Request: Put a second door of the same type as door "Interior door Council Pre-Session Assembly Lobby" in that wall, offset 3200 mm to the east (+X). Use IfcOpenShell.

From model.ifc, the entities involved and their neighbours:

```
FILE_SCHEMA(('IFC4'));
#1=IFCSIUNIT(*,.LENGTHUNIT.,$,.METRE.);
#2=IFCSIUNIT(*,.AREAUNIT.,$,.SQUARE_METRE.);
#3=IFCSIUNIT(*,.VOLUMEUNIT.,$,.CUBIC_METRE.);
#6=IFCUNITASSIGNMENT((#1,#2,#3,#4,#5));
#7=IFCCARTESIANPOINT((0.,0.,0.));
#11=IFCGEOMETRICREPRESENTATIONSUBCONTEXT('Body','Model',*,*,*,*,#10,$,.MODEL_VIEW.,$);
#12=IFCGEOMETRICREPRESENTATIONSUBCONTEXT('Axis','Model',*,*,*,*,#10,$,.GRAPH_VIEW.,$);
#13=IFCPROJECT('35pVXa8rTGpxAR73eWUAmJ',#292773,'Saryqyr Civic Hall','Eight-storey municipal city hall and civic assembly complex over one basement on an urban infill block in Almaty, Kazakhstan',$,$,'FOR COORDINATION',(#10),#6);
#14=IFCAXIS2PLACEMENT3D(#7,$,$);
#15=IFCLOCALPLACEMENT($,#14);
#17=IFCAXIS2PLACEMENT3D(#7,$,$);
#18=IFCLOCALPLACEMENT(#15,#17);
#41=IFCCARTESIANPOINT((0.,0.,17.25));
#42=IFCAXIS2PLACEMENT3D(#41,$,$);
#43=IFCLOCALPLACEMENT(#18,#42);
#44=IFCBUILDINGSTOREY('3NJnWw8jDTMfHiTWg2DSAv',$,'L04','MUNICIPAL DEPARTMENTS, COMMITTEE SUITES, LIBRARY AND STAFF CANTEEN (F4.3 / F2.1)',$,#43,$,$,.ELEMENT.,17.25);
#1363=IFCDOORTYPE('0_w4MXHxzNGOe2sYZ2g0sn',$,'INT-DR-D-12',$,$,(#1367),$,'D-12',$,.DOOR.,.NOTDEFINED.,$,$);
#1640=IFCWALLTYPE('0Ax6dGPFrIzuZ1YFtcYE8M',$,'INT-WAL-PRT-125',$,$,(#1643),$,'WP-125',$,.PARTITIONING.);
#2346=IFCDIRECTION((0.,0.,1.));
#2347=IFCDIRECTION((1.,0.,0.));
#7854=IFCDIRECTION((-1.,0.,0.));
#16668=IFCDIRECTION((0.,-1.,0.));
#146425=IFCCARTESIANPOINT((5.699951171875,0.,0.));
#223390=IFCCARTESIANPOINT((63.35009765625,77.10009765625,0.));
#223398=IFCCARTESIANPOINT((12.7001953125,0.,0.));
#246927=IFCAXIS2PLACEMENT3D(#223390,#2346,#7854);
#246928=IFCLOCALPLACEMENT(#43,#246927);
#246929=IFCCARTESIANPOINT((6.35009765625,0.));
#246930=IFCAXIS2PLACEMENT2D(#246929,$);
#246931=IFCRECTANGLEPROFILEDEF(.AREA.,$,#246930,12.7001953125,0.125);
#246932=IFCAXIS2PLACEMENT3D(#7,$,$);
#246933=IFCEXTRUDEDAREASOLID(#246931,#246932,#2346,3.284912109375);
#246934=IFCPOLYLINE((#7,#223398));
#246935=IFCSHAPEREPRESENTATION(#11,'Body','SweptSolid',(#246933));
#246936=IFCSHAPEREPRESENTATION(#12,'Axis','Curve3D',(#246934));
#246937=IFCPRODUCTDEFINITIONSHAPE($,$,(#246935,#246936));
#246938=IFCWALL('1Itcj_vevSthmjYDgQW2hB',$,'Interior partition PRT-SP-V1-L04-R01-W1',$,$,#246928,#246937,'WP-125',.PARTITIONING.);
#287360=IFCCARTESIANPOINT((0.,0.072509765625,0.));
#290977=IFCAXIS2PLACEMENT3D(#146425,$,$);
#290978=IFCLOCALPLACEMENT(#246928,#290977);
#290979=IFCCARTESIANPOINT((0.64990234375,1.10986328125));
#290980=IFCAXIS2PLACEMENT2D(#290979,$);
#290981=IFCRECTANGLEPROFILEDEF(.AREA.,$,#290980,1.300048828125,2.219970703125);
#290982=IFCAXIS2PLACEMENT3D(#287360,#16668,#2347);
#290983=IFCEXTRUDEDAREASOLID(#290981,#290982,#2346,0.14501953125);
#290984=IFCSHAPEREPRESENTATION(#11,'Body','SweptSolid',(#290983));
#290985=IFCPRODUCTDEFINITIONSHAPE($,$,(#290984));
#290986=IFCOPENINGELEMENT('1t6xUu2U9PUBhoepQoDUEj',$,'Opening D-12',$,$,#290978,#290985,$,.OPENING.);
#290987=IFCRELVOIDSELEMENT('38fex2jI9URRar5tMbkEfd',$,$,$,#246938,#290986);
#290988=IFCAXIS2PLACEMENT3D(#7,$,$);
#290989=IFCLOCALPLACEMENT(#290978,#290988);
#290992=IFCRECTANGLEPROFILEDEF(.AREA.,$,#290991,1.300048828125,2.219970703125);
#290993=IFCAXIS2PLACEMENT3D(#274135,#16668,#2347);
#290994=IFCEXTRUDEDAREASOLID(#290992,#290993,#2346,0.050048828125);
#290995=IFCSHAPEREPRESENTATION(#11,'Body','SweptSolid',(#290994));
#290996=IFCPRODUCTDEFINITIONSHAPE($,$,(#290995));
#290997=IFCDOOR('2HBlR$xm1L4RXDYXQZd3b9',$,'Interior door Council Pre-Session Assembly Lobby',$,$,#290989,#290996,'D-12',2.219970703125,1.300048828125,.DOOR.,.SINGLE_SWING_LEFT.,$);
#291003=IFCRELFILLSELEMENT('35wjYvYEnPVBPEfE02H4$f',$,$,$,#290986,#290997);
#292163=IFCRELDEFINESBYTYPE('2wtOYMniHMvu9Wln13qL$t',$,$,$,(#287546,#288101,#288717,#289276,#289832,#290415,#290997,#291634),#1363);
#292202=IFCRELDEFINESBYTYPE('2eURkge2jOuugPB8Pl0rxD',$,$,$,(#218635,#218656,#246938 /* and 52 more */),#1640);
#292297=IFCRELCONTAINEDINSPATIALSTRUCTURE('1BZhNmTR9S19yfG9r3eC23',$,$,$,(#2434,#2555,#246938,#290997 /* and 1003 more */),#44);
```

```python
import ifcopenshell
import ifcopenshell.api.feature
import ifcopenshell.api.geometry
import ifcopenshell.api.root
import ifcopenshell.geom
import ifcopenshell.util.element
import ifcopenshell.util.placement
import ifcopenshell.util.shape
import ifcopenshell.util.unit

model = ifcopenshell.open("model.ifc")
unit_scale = ifcopenshell.util.unit.calculate_unit_scale(model)
settings = ifcopenshell.geom.settings()


def volume(element):
    """Net volume in cubic metres, openings subtracted."""
    shape = ifcopenshell.geom.create_shape(settings, element)
    return ifcopenshell.util.shape.get_volume(shape.geometry)


door = model.by_guid("2HBlR$xm1L4RXDYXQZd3b9")
opening = door.FillsVoids[0].RelatingOpeningElement
wall = opening.VoidsElements[0].RelatingBuildingElement
before = volume(wall)
shift = ifcopenshell.util.placement.get_local_placement(wall.ObjectPlacement)[:3, 0] * -3.2 / unit_scale

# copy_class copies the void relationship, type, container and properties, but no geometry.
new_opening = ifcopenshell.api.root.copy_class(model, product=opening)
new_opening.Representation = ifcopenshell.util.element.copy_deep(
    model, opening.Representation, exclude=["IfcGeometricRepresentationContext", "IfcRepresentationMap"]
)
new_door = ifcopenshell.api.root.copy_class(model, product=door)
new_door.Representation = ifcopenshell.util.element.copy_deep(
    model, door.Representation, exclude=["IfcGeometricRepresentationContext", "IfcRepresentationMap"]
)
new_door.Tag = None
ifcopenshell.api.feature.add_filling(model, opening=new_opening, element=new_door)

for old, new in ((opening, new_opening), (door, new_door)):
    matrix = ifcopenshell.util.placement.get_local_placement(old.ObjectPlacement)
    matrix[:3, 3] += shift
    ifcopenshell.api.geometry.edit_object_placement(model, product=new, matrix=matrix, is_si=False)

after = volume(wall)

print(f"wall volume {before:.3f} -> {after:.3f} m3")

model.write("model_v2.ifc")
```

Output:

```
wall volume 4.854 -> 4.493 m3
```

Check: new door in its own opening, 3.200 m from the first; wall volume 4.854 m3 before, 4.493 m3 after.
